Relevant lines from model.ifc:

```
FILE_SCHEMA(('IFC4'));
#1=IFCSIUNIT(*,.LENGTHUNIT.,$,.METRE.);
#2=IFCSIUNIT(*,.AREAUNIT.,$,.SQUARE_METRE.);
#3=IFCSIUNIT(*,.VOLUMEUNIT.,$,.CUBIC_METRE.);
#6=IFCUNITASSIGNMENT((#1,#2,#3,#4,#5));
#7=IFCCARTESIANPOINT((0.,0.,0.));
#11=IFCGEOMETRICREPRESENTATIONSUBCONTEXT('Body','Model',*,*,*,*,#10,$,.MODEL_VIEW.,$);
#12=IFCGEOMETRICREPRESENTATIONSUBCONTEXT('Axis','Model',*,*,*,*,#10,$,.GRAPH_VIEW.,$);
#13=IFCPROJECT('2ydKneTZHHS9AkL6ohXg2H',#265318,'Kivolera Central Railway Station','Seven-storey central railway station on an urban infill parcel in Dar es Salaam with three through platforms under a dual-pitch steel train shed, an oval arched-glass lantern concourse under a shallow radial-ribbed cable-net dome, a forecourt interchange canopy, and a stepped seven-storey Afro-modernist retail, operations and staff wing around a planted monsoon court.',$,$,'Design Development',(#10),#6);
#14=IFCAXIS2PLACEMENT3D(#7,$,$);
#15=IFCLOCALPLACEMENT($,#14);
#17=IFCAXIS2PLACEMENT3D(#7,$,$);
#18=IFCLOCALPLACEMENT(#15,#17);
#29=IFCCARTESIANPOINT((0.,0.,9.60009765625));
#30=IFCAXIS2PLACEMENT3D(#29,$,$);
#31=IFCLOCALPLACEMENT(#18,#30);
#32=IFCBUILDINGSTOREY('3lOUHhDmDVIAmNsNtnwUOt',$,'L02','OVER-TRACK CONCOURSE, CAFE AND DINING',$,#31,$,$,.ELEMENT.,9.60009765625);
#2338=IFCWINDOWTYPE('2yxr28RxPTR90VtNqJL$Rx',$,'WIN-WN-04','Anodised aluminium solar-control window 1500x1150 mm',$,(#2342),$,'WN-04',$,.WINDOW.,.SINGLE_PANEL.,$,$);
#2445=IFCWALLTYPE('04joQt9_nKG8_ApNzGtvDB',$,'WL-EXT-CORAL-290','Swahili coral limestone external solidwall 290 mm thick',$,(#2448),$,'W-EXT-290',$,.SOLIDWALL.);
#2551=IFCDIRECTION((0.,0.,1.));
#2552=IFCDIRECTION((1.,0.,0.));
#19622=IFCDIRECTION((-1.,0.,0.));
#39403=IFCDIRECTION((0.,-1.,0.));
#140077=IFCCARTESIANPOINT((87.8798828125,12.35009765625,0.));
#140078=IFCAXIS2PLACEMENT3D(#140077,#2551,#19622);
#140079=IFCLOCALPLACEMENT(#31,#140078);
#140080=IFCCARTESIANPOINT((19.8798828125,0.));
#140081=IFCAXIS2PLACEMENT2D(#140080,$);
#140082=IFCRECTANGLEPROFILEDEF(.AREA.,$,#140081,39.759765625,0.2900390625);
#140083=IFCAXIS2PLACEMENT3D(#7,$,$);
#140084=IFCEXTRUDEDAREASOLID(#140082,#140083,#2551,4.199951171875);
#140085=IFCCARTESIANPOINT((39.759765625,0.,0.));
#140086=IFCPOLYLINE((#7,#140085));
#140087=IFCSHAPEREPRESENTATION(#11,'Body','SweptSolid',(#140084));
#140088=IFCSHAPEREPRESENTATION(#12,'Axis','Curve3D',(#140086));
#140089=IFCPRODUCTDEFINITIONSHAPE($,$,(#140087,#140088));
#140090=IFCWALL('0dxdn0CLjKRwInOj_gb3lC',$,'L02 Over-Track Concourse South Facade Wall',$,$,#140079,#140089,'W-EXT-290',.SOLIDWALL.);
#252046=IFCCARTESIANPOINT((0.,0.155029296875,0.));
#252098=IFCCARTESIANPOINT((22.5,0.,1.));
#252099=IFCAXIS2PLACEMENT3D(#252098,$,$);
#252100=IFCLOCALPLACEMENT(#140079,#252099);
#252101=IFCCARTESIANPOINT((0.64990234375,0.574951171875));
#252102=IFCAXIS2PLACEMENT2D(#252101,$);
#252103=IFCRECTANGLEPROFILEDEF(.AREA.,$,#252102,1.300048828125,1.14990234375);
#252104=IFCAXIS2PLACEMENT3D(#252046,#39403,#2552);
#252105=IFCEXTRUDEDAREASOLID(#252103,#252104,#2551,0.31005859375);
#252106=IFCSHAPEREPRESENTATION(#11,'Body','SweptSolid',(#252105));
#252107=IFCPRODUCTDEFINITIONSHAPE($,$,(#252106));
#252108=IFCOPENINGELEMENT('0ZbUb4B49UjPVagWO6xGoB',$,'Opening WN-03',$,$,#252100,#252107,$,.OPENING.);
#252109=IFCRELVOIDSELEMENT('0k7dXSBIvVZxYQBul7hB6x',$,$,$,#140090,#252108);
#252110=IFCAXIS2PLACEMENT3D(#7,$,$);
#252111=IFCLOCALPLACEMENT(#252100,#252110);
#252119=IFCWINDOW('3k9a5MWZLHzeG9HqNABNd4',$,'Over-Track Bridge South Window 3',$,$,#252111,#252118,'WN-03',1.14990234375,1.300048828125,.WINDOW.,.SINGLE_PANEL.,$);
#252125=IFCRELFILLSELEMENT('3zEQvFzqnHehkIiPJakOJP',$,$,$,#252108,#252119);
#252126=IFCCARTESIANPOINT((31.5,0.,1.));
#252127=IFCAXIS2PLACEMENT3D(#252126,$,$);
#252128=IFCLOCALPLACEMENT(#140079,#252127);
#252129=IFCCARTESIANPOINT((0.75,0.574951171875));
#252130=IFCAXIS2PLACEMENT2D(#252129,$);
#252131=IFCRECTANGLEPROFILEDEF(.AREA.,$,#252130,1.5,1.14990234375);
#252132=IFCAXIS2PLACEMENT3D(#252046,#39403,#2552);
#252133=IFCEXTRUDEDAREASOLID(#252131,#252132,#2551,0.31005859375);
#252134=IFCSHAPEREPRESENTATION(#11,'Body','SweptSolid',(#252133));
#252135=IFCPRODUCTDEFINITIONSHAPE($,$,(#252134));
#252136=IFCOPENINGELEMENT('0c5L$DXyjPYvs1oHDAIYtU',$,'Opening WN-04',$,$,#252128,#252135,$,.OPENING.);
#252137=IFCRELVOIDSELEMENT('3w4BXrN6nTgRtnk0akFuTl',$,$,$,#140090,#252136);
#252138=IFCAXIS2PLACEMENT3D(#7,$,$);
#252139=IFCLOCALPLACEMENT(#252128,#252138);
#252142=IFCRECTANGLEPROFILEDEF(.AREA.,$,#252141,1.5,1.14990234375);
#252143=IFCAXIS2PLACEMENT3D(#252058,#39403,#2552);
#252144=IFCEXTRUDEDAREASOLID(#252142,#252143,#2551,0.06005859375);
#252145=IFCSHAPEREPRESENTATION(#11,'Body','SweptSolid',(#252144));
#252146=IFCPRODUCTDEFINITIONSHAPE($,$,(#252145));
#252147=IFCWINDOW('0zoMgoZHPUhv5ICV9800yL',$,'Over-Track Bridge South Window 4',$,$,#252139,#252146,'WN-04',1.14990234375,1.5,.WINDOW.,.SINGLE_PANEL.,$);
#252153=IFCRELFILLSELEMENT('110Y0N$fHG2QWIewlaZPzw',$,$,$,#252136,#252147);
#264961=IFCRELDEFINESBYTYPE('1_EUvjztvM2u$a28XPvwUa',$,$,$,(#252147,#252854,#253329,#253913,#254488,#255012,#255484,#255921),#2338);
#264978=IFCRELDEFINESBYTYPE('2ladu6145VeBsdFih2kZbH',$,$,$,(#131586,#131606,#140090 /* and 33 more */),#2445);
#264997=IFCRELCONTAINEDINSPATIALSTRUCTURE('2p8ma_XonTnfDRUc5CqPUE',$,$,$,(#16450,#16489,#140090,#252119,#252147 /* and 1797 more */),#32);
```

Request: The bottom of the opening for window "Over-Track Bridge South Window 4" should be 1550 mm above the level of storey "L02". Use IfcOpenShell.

```python
import numpy as np
import ifcopenshell
import ifcopenshell.api.geometry
import ifcopenshell.geom
import ifcopenshell.util.element
import ifcopenshell.util.placement
import ifcopenshell.util.shape
import ifcopenshell.util.unit

model = ifcopenshell.open("model.ifc")
unit_scale = ifcopenshell.util.unit.calculate_unit_scale(model)

window = model.by_guid("0zoMgoZHPUhv5ICV9800yL")
opening = window.FillsVoids[0].RelatingOpeningElement
storey = ifcopenshell.util.element.get_container(window, ifc_class="IfcBuildingStorey")
level = ifcopenshell.util.placement.get_local_placement(storey.ObjectPlacement)[2, 3]

# The opening's origin need not be at the sill, so measure its lowest point.
shape = ifcopenshell.geom.create_shape(ifcopenshell.geom.settings(), opening)
bottom = ifcopenshell.util.shape.get_shape_bottom_elevation(shape, shape.geometry) / unit_scale
dz = level + 1.55 / unit_scale - bottom

shift = np.array([0.0, 0.0, dz])
# The window is placed relative to its opening, so it follows when the opening moves.
matrix = ifcopenshell.util.placement.get_local_placement(opening.ObjectPlacement)
matrix[:3, 3] += shift
ifcopenshell.api.geometry.edit_object_placement(
    model, product=opening, matrix=matrix, is_si=False, should_transform_children=True
)

print(f"moved by {dz * unit_scale:+.3f} m")

model.write("model_edited.ifc")
```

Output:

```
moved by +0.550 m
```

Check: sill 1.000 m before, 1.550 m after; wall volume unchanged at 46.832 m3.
